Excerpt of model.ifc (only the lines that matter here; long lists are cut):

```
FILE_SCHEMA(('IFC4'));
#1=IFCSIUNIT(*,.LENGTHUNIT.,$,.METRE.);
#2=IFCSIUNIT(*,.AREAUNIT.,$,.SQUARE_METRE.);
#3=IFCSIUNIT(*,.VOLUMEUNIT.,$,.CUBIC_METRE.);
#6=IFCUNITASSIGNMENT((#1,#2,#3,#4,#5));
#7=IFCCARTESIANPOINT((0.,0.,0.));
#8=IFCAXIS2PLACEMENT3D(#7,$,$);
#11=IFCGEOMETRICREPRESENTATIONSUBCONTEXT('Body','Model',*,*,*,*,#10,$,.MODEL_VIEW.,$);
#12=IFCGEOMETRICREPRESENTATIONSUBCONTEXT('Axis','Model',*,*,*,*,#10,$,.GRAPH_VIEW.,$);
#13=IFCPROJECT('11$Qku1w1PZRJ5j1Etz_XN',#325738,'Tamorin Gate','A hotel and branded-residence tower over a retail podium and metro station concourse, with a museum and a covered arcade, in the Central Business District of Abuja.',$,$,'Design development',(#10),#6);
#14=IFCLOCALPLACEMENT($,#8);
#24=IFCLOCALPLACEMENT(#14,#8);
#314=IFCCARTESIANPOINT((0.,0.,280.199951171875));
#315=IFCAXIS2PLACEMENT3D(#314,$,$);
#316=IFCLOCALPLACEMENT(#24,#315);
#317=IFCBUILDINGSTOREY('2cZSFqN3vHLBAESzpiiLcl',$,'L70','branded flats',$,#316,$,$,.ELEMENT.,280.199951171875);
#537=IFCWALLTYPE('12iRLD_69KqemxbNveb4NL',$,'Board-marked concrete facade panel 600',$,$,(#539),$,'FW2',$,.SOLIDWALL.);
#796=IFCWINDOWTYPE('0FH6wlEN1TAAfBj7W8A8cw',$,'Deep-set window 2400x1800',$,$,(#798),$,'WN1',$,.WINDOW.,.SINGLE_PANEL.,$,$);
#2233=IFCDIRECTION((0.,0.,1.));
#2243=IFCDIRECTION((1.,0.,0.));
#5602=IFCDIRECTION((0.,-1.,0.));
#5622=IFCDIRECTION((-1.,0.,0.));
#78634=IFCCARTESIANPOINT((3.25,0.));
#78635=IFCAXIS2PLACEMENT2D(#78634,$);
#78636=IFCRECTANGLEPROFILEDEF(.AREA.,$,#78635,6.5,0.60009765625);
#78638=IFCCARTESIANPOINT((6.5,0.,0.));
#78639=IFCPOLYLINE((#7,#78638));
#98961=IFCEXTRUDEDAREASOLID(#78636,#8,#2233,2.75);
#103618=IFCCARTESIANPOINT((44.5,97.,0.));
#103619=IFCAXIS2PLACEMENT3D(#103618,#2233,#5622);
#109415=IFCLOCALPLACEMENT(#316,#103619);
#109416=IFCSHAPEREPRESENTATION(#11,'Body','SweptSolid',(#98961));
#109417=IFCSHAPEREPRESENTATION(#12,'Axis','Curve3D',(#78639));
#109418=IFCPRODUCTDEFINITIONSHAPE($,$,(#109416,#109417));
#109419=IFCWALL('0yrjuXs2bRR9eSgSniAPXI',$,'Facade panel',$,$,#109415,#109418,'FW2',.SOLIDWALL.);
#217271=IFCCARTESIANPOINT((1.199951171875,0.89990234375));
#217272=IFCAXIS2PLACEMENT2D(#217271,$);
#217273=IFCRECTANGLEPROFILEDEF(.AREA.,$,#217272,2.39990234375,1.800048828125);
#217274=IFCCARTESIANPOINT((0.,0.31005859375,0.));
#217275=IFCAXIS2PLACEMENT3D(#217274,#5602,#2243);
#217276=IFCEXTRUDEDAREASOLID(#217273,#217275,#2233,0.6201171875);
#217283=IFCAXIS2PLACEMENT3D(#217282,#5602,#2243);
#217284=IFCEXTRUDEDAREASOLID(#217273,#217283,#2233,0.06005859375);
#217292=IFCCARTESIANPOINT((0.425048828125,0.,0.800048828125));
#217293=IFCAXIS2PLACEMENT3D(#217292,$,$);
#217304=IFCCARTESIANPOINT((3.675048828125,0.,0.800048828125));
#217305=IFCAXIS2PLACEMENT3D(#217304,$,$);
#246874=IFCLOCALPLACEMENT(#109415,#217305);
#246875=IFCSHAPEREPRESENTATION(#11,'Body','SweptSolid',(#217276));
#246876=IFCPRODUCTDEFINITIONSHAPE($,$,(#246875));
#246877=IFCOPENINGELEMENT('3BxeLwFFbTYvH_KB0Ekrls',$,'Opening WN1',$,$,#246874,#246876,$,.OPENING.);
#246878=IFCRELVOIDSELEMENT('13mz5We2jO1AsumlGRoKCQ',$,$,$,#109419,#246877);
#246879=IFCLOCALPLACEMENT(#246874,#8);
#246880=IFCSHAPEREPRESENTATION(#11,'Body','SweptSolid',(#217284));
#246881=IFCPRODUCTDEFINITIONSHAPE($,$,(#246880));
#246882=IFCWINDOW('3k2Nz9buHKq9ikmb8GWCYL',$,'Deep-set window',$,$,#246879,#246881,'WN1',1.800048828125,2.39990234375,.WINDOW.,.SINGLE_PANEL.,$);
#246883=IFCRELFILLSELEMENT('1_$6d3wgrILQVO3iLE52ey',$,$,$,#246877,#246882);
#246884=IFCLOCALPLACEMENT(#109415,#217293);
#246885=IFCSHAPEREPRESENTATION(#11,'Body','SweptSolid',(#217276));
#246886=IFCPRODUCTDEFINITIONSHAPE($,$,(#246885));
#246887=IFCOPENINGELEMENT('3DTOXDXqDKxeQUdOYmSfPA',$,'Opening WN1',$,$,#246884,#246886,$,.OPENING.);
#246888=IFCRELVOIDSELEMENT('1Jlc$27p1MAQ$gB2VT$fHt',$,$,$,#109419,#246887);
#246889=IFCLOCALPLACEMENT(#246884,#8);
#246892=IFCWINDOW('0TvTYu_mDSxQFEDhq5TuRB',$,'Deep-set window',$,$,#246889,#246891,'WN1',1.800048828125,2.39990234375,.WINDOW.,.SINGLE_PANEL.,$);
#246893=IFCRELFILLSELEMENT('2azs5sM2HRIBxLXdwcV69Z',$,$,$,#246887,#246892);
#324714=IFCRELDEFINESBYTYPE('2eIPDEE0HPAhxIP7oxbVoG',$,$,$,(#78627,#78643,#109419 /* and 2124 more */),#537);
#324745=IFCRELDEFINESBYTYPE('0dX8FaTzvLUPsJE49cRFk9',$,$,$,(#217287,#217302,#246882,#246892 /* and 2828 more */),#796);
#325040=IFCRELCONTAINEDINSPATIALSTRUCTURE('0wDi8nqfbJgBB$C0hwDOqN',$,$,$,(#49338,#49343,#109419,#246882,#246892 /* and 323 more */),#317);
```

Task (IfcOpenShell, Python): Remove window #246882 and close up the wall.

```python
import ifcopenshell
import ifcopenshell.api.feature
import ifcopenshell.api.root
import ifcopenshell.geom
import ifcopenshell.util.shape

model = ifcopenshell.open("model.ifc")
settings = ifcopenshell.geom.settings()


def volume(element):
    """Net volume in cubic metres, openings subtracted."""
    shape = ifcopenshell.geom.create_shape(settings, element)
    return ifcopenshell.util.shape.get_volume(shape.geometry)


window = model.by_id(246882)
opening = window.FillsVoids[0].RelatingOpeningElement
wall = opening.VoidsElements[0].RelatingBuildingElement
before = volume(wall)

ifcopenshell.api.root.remove_product(model, product=window)
ifcopenshell.api.feature.remove_feature(model, feature=opening)

after = volume(wall)

print(f"wall volume {before:.3f} -> {after:.3f} m3")

model.write("model_rev.ifc")
```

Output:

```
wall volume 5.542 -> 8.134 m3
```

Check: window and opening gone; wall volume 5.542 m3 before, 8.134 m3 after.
